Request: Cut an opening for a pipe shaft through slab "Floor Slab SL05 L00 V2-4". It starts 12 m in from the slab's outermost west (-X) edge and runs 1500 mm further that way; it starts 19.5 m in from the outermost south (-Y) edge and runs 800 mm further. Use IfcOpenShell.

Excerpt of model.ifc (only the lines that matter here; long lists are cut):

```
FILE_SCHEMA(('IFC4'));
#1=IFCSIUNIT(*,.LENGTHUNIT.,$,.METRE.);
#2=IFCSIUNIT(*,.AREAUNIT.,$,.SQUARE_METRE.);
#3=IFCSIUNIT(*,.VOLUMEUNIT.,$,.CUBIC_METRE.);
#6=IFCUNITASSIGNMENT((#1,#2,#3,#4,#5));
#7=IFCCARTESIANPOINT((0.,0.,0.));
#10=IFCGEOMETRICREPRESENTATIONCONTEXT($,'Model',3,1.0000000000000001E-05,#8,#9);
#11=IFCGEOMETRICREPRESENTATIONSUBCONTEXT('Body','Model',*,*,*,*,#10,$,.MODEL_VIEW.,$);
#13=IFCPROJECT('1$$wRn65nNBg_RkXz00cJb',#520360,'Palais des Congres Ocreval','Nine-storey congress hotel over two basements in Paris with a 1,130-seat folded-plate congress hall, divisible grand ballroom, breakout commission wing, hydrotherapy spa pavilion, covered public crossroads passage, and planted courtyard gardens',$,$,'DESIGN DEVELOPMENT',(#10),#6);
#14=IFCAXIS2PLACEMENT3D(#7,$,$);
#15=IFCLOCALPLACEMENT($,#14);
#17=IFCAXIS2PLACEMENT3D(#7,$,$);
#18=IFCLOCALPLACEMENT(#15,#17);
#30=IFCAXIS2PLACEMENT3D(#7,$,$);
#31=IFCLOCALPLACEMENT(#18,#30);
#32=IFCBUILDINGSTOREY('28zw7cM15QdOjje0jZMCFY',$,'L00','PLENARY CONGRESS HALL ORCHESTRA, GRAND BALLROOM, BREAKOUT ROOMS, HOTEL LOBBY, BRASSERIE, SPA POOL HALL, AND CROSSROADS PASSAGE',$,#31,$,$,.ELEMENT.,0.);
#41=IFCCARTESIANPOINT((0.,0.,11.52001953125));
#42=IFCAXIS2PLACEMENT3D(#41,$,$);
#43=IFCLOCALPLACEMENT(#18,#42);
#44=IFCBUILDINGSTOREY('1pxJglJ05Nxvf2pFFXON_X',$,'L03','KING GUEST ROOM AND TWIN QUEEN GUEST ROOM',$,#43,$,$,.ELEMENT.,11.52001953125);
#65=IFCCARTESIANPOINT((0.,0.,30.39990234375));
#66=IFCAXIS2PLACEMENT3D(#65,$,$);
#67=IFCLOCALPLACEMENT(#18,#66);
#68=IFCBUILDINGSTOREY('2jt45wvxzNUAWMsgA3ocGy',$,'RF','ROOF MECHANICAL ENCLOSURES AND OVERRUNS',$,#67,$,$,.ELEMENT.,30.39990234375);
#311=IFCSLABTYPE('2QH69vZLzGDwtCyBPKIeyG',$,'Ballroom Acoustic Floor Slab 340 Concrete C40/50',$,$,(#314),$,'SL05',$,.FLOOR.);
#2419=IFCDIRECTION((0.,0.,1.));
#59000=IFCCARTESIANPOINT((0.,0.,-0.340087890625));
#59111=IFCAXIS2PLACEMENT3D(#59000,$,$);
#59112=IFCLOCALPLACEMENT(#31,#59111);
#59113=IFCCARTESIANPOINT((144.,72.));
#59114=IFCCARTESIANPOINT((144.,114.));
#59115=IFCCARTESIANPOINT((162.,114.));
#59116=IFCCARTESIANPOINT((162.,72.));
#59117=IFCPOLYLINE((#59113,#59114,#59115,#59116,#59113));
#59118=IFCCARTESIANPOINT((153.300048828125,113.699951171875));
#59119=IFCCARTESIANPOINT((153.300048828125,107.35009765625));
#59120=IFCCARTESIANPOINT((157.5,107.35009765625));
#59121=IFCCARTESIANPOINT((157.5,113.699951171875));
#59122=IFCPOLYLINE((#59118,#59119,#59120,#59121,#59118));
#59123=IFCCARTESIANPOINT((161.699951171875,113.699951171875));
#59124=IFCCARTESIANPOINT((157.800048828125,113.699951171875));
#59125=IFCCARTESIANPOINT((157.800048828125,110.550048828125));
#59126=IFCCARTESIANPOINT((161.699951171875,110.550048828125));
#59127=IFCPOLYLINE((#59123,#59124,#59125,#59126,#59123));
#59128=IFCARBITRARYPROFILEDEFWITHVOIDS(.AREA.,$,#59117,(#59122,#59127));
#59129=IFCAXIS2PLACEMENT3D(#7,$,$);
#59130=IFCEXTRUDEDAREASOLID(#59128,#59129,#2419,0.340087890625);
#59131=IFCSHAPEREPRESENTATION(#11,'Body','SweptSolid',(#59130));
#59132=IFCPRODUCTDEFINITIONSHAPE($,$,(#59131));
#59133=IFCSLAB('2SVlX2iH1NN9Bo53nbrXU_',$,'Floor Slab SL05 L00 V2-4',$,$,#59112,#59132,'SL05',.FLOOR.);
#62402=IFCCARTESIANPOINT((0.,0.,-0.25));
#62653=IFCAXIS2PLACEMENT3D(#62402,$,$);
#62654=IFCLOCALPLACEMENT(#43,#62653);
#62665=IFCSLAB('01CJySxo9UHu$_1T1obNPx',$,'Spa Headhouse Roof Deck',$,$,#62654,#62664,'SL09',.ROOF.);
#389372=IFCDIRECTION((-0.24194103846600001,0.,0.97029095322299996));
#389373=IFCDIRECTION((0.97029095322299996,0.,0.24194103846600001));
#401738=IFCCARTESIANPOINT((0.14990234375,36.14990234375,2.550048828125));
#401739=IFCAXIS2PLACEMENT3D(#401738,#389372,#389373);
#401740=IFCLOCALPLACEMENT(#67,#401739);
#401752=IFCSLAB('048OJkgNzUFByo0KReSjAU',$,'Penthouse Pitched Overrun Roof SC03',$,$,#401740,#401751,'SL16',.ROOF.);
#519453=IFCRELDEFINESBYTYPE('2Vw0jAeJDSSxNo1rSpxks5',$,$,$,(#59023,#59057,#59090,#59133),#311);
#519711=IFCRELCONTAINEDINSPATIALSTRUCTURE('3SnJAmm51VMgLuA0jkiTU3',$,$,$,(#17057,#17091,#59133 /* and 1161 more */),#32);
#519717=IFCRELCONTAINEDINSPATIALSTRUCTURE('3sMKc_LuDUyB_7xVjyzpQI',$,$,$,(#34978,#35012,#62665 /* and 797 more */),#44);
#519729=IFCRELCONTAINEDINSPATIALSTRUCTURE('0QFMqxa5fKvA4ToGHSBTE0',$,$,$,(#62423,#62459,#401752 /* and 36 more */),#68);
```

```python
import numpy as np
import ifcopenshell
import ifcopenshell.api.feature
import ifcopenshell.api.geometry
import ifcopenshell.api.root
import ifcopenshell.geom
import ifcopenshell.util.placement
import ifcopenshell.util.representation
import ifcopenshell.util.shape
import ifcopenshell.util.unit

model = ifcopenshell.open("model.ifc")
unit_scale = ifcopenshell.util.unit.calculate_unit_scale(model)
settings = ifcopenshell.geom.settings()


def volume(element):
    """Net volume in cubic metres, openings subtracted."""
    shape = ifcopenshell.geom.create_shape(settings, element)
    return ifcopenshell.util.shape.get_volume(shape.geometry)


slab = model.by_guid("2SVlX2iH1NN9Bo53nbrXU_")
before = volume(slab)

# Extent in the slab's own axes, in metres. The edges named are its -X and -Y sides.
slab_shape = ifcopenshell.geom.create_shape(settings, slab)
vertices = ifcopenshell.util.shape.get_vertices(slab_shape.geometry)
x_min, y_min, bottom = vertices.min(axis=0)
top = vertices[:, 2].max()

opening = ifcopenshell.api.root.create_entity(model, ifc_class="IfcOpeningElement", name="Pipe shaft opening", predefined_type="OPENING")
context = ifcopenshell.util.representation.get_context(model, "Model", "Body", "MODEL_VIEW")
width, depth = 1.5, 0.8
outline = [(0.0, 0.0), (width, 0.0), (width, depth), (0.0, depth), (0.0, 0.0)]
# Overshoot both faces by 50 mm so the cut is clean.
shape = ifcopenshell.api.geometry.add_slab_representation(
    model, context=context, depth=top - bottom + 0.1, polyline=outline
)
ifcopenshell.api.geometry.assign_representation(model, product=opening, representation=shape)

matrix = ifcopenshell.util.placement.get_local_placement(slab.ObjectPlacement)
matrix[:, 3] = matrix @ np.append(np.array([x_min + 12, y_min + 19.5, bottom - 0.05]) / unit_scale, 1.0)
ifcopenshell.api.geometry.edit_object_placement(model, product=opening, matrix=matrix, is_si=False)
ifcopenshell.api.feature.add_feature(model, feature=opening, element=slab)

after = volume(slab)

print(f"slab volume {before:.3f} -> {after:.3f} m3")

model.write("model_updated.ifc")
```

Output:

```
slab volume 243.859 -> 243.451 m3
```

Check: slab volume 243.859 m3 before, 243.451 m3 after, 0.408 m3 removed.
